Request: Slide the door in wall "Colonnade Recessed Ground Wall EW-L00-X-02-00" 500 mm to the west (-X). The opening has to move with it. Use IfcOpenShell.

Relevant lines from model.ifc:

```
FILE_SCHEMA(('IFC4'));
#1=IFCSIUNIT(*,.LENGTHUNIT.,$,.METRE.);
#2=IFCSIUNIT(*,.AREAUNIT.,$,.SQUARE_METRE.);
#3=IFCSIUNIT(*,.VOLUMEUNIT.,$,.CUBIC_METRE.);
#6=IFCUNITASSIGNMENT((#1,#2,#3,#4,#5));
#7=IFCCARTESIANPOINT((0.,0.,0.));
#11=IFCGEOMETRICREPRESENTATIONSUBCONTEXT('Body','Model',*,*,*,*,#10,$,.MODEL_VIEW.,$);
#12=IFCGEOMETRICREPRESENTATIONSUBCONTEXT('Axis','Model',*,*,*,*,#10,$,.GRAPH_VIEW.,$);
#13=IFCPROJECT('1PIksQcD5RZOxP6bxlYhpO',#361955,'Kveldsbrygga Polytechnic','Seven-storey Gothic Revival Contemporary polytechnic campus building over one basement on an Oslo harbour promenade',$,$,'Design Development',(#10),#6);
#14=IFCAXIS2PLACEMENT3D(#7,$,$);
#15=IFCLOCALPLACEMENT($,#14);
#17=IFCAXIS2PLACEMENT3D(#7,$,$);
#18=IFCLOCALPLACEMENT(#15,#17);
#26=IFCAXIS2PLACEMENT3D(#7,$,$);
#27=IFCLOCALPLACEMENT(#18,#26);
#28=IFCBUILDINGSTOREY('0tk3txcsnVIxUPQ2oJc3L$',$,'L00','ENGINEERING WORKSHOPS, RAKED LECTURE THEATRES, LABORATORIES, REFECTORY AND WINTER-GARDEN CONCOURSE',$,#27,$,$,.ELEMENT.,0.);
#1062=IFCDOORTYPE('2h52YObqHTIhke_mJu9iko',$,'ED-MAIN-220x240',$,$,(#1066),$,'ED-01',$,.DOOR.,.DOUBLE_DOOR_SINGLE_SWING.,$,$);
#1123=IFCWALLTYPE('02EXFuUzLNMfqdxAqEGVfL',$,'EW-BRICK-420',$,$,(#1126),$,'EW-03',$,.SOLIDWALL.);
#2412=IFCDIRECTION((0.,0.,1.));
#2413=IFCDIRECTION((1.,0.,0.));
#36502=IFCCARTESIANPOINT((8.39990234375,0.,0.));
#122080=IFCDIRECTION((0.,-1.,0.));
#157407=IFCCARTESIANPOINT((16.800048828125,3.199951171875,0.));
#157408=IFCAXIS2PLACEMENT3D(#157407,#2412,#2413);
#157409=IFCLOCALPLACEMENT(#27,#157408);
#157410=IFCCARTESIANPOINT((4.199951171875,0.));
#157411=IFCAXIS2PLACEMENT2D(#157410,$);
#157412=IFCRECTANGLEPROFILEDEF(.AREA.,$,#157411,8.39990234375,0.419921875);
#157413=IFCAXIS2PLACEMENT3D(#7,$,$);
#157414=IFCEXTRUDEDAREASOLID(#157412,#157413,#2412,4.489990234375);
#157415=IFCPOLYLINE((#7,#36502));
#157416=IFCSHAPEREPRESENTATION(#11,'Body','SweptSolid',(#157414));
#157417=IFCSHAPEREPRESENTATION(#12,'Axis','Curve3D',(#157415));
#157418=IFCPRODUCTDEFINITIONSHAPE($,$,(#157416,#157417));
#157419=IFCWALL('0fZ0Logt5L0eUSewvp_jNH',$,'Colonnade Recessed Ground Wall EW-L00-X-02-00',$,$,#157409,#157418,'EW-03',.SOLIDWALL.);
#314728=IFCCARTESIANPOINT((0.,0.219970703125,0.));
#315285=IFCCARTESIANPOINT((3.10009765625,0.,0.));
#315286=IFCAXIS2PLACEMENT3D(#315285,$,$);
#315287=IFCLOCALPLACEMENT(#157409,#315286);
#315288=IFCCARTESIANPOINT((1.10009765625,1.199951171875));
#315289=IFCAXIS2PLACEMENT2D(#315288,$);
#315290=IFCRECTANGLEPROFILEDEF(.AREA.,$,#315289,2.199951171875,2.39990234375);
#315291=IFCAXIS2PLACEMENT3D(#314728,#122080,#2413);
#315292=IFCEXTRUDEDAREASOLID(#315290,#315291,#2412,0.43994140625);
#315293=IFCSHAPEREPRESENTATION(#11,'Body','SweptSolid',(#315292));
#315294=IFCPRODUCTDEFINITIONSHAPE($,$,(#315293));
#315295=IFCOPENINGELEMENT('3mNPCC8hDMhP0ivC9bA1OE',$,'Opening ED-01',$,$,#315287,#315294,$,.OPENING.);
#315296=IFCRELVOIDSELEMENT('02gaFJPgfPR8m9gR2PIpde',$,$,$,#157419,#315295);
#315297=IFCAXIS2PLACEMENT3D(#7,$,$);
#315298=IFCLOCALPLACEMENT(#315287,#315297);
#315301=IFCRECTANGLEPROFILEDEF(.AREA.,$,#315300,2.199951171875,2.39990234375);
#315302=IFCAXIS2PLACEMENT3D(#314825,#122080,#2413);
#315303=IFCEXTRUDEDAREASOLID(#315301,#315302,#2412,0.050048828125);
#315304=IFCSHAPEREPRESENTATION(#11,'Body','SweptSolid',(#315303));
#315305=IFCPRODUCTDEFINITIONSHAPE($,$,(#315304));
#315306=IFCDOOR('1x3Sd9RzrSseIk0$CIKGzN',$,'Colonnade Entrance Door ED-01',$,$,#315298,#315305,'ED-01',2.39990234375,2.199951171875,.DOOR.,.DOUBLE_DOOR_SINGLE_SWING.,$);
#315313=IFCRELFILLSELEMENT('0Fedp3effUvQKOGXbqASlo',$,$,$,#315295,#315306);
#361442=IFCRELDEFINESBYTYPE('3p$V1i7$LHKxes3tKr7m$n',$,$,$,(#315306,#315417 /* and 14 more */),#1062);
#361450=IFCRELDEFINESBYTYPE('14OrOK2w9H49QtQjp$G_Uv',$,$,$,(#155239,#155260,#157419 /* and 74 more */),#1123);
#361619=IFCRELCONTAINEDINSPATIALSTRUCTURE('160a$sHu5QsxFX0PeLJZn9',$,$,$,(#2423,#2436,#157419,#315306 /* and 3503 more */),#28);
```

```python
import ifcopenshell
import ifcopenshell.api.geometry
import ifcopenshell.util.placement
import ifcopenshell.util.unit

model = ifcopenshell.open("model.ifc")
unit_scale = ifcopenshell.util.unit.calculate_unit_scale(model)

door = model.by_guid("1x3Sd9RzrSseIk0$CIKGzN")
opening = door.FillsVoids[0].RelatingOpeningElement
wall = opening.VoidsElements[0].RelatingBuildingElement

wall_matrix = ifcopenshell.util.placement.get_local_placement(wall.ObjectPlacement)
shift = wall_matrix[:3, 0] * -0.5 / unit_scale
before = ifcopenshell.util.placement.get_local_placement(door.ObjectPlacement)[:3, 3].copy()

# The door is placed relative to its opening, so it follows when the opening moves.
matrix = ifcopenshell.util.placement.get_local_placement(opening.ObjectPlacement)
matrix[:3, 3] += shift
ifcopenshell.api.geometry.edit_object_placement(
    model, product=opening, matrix=matrix, is_si=False, should_transform_children=True
)

after = ifcopenshell.util.placement.get_local_placement(door.ObjectPlacement)[:3, 3]
print("door moved by", (after - before).round(3) + 0.0)

model.write("model_v2.ifc")
```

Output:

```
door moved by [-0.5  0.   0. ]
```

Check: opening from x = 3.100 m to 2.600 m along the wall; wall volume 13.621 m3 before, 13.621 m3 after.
